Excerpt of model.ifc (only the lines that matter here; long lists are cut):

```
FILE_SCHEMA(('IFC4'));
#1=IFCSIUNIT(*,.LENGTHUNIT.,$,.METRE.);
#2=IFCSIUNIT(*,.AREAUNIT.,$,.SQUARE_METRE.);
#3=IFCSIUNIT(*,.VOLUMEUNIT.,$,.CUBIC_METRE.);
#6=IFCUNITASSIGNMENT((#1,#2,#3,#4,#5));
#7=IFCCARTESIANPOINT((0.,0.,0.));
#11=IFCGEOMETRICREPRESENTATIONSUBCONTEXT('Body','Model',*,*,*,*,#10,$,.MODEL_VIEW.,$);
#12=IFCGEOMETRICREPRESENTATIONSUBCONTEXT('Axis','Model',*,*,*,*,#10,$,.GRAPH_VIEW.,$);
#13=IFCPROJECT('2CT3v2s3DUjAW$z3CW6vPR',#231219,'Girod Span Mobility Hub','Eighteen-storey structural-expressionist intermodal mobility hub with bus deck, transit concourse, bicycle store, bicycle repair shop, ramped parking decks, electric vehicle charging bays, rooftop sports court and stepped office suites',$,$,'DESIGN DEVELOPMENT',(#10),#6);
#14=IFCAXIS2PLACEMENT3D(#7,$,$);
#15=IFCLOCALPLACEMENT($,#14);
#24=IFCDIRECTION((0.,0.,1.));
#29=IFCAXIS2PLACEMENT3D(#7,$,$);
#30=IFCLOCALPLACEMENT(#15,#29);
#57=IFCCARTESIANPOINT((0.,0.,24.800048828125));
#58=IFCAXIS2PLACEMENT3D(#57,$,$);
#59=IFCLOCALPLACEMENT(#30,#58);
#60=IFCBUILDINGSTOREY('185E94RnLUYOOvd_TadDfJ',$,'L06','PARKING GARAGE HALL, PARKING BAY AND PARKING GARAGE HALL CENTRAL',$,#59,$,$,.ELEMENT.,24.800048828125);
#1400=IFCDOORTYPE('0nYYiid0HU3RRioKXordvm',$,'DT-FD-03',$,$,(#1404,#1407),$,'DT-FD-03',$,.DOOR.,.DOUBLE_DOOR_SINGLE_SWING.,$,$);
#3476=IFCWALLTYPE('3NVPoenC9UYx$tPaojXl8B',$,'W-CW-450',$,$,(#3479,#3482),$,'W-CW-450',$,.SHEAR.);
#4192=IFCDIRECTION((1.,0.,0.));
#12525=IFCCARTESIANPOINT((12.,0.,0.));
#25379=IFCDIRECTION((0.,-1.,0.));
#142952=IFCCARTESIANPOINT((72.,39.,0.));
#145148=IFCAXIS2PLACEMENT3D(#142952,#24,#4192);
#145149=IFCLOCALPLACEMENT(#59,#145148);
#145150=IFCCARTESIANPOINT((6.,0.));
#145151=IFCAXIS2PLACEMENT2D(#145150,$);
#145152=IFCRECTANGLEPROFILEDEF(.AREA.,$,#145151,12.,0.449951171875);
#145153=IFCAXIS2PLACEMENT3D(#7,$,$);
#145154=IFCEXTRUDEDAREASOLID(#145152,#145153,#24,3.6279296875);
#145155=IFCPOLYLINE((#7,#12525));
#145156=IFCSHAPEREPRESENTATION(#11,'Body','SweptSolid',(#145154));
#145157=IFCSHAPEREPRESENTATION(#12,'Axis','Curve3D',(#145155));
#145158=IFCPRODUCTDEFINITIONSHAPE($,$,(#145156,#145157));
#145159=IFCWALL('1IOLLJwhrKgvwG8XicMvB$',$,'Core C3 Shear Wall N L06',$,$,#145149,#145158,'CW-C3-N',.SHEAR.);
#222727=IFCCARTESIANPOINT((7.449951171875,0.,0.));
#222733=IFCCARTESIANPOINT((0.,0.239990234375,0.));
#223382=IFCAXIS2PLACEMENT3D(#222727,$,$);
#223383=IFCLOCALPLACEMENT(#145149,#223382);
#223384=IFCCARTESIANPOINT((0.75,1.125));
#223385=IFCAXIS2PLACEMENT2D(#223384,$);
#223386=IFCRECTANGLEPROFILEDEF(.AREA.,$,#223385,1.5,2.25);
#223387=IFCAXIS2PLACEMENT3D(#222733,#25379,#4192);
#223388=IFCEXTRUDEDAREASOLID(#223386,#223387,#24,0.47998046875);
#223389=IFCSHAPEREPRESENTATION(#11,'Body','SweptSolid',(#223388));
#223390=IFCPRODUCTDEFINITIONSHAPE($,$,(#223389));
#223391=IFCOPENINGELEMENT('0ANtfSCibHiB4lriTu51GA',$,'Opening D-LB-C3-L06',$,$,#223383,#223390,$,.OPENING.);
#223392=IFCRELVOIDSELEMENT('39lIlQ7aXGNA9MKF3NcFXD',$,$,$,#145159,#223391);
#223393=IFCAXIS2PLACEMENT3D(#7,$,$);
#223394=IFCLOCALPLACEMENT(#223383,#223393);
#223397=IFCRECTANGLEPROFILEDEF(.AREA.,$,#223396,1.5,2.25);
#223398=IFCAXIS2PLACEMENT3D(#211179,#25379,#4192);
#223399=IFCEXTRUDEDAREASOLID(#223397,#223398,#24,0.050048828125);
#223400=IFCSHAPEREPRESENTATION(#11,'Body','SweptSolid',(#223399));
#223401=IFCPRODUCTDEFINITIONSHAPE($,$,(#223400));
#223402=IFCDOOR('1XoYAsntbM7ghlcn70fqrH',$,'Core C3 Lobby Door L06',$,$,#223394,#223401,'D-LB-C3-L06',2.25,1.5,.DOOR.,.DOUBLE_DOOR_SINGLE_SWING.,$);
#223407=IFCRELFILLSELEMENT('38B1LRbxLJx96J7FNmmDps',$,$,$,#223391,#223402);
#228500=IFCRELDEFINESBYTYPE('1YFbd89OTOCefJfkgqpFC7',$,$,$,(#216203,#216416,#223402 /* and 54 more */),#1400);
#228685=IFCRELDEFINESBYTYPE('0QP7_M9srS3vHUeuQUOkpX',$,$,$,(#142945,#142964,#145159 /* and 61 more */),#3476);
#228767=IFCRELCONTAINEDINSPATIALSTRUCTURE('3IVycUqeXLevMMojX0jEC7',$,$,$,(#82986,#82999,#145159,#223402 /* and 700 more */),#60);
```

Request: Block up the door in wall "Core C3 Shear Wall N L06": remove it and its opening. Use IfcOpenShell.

```python
import ifcopenshell
import ifcopenshell.api.feature
import ifcopenshell.api.root
import ifcopenshell.geom
import ifcopenshell.util.shape

model = ifcopenshell.open("model.ifc")
settings = ifcopenshell.geom.settings()


def volume(element):
    """Net volume in cubic metres, openings subtracted."""
    shape = ifcopenshell.geom.create_shape(settings, element)
    return ifcopenshell.util.shape.get_volume(shape.geometry)


door = model.by_guid("1XoYAsntbM7ghlcn70fqrH")
opening = door.FillsVoids[0].RelatingOpeningElement
wall = opening.VoidsElements[0].RelatingBuildingElement
before = volume(wall)

ifcopenshell.api.root.remove_product(model, product=door)
ifcopenshell.api.feature.remove_feature(model, feature=opening)

after = volume(wall)

print(f"wall volume {before:.3f} -> {after:.3f} m3")

model.write("model_v2.ifc")
```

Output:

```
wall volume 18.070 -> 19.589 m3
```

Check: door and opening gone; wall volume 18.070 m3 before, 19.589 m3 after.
